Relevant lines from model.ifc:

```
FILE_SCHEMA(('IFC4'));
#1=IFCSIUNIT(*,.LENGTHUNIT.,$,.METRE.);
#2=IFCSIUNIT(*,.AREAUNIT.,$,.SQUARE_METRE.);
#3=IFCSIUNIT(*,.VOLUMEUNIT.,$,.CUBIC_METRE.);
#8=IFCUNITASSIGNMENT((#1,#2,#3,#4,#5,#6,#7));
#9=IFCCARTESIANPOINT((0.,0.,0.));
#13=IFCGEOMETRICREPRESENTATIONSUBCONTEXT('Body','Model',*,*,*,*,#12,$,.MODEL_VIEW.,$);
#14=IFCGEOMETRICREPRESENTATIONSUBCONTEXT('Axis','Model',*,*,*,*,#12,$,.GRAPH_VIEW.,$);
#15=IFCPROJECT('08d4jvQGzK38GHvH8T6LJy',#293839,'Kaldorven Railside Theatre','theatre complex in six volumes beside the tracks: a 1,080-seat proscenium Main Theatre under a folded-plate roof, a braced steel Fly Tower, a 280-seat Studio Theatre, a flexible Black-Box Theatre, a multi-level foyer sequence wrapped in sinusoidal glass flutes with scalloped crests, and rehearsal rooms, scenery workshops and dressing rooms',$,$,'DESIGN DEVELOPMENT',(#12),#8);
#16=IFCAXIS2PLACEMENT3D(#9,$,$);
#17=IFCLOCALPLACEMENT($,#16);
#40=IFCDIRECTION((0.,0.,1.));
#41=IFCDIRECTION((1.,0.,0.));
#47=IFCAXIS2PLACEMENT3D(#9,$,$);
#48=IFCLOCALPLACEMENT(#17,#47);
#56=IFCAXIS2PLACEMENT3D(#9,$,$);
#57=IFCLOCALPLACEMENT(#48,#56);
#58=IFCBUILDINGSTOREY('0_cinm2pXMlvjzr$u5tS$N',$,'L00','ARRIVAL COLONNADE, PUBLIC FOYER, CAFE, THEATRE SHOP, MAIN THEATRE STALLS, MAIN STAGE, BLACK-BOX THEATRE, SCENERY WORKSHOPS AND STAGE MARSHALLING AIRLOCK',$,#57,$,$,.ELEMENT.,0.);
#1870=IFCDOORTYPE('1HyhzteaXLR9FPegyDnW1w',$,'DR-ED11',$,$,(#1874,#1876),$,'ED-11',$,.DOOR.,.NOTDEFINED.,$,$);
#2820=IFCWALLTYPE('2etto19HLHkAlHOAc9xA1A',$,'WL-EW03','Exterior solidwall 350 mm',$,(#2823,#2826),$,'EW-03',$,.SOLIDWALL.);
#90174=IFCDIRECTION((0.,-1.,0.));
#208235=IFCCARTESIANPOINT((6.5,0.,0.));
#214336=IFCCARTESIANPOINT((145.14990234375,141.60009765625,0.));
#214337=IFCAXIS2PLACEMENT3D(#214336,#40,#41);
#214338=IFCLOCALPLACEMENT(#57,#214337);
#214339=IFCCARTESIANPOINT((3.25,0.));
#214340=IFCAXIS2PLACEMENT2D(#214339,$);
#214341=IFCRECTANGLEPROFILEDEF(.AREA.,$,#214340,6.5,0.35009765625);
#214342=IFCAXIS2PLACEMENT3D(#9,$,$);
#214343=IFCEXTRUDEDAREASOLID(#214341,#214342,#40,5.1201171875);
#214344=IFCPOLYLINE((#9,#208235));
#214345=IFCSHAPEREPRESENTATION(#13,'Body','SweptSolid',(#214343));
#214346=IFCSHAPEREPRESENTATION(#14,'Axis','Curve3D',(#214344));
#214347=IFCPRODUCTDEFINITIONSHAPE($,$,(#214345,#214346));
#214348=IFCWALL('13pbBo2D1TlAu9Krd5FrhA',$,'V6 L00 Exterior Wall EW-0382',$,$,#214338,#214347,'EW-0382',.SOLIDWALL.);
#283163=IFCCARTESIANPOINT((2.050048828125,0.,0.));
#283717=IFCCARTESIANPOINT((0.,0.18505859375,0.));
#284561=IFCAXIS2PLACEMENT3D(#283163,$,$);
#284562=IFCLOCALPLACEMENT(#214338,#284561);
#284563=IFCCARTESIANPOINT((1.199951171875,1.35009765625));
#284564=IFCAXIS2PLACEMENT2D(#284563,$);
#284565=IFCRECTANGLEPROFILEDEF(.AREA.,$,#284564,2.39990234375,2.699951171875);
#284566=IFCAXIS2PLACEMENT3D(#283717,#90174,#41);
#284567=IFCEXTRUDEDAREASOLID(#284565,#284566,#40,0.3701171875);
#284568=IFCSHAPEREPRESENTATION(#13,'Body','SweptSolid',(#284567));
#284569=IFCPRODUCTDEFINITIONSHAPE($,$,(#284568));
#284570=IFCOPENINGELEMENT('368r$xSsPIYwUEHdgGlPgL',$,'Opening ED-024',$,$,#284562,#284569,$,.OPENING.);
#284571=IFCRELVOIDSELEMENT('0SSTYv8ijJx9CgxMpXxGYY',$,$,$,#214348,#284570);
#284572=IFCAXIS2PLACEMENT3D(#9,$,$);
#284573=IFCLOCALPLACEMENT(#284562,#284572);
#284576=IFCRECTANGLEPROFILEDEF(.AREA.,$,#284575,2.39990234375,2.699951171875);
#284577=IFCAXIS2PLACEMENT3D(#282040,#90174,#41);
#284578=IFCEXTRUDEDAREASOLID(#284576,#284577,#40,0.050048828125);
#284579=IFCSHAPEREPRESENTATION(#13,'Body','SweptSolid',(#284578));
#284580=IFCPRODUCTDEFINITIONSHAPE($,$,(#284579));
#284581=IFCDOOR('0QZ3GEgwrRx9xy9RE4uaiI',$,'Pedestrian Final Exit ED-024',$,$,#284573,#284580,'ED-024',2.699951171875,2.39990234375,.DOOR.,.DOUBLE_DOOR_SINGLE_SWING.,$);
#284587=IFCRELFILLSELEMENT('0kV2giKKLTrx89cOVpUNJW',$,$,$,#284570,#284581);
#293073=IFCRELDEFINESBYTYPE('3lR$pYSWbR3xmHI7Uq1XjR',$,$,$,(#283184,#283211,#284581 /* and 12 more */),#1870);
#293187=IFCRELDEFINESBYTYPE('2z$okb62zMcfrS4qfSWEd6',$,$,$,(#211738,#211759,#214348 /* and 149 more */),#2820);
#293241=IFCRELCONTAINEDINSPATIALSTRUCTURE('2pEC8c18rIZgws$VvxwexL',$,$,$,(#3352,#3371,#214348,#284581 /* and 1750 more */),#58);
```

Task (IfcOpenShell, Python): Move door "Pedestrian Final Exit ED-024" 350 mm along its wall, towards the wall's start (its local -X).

```python
import ifcopenshell
import ifcopenshell.api.geometry
import ifcopenshell.util.placement
import ifcopenshell.util.unit

model = ifcopenshell.open("model.ifc")
unit_scale = ifcopenshell.util.unit.calculate_unit_scale(model)

door = model.by_id(284581)
opening = door.FillsVoids[0].RelatingOpeningElement
wall = opening.VoidsElements[0].RelatingBuildingElement

wall_matrix = ifcopenshell.util.placement.get_local_placement(wall.ObjectPlacement)
shift = wall_matrix[:3, 0] * -0.35 / unit_scale
before = ifcopenshell.util.placement.get_local_placement(door.ObjectPlacement)[:3, 3].copy()

# The door is placed relative to its opening, so it follows when the opening moves.
matrix = ifcopenshell.util.placement.get_local_placement(opening.ObjectPlacement)
matrix[:3, 3] += shift
ifcopenshell.api.geometry.edit_object_placement(
    model, product=opening, matrix=matrix, is_si=False, should_transform_children=True
)

after = ifcopenshell.util.placement.get_local_placement(door.ObjectPlacement)[:3, 3]
print("door moved by", (after - before).round(3) + 0.0)

model.write("model_updated.ifc")
```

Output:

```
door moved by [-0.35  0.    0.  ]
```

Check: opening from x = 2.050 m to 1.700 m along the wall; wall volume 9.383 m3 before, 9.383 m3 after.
